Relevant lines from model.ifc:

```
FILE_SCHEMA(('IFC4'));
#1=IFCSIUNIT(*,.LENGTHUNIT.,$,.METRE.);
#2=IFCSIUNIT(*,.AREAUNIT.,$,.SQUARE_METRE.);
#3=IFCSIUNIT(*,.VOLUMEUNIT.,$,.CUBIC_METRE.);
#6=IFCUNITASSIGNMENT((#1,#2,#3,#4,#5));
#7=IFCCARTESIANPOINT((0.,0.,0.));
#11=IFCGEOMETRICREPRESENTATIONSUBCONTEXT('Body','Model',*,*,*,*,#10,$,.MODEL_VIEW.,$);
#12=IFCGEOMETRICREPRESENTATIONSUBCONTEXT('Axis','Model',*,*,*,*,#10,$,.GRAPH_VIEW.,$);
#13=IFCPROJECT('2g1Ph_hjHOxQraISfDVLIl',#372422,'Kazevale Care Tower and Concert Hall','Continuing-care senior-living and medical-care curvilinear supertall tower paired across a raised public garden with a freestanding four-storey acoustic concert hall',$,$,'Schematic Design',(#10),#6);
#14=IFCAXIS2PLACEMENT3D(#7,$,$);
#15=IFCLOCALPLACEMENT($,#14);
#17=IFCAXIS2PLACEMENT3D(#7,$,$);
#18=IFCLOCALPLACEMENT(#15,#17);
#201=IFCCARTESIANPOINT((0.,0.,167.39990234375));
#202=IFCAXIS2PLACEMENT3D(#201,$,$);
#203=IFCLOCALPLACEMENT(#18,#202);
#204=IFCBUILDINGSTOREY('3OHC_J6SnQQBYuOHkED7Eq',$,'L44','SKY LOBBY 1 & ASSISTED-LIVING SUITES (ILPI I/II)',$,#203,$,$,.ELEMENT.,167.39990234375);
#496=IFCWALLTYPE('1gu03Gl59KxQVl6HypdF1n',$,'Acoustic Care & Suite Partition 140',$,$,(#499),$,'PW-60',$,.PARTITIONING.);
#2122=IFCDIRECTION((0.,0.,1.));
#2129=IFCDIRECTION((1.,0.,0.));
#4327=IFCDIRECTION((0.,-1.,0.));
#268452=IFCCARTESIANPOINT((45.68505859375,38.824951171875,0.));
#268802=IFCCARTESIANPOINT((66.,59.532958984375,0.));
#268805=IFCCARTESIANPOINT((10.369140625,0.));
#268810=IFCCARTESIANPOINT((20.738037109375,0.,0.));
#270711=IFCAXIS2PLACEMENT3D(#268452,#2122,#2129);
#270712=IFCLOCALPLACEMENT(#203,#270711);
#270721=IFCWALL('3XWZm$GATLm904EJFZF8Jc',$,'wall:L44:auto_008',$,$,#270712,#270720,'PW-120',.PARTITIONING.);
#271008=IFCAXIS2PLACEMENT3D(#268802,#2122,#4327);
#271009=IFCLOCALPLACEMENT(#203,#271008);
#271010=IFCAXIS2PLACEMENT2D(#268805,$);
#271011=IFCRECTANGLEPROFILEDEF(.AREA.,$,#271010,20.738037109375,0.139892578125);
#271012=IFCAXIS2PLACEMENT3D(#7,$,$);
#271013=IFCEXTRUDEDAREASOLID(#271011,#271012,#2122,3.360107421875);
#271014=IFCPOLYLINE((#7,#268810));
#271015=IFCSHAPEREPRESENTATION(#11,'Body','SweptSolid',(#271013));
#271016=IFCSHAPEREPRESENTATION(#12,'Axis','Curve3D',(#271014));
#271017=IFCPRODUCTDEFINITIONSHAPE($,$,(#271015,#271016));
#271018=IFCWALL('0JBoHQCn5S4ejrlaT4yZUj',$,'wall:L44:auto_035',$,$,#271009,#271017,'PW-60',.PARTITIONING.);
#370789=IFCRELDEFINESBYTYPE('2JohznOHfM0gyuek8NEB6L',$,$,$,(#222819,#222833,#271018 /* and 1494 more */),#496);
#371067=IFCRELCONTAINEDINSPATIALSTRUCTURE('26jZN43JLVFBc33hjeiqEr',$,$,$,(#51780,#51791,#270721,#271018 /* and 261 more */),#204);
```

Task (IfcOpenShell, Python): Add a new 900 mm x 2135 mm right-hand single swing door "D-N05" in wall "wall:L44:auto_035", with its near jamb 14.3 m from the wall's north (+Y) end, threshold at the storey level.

```python
import numpy as np
import ifcopenshell
import ifcopenshell.api.feature
import ifcopenshell.api.geometry
import ifcopenshell.api.root
import ifcopenshell.api.spatial
import ifcopenshell.geom
import ifcopenshell.util.element
import ifcopenshell.util.placement
import ifcopenshell.util.representation
import ifcopenshell.util.shape
import ifcopenshell.util.unit

model = ifcopenshell.open("model.ifc")
unit_scale = ifcopenshell.util.unit.calculate_unit_scale(model)
settings = ifcopenshell.geom.settings()


def volume(element):
    """Net volume in cubic metres, openings subtracted."""
    shape = ifcopenshell.geom.create_shape(settings, element)
    return ifcopenshell.util.shape.get_volume(shape.geometry)


wall = model.by_id(271018)
storey = ifcopenshell.util.element.get_container(wall, ifc_class="IfcBuildingStorey")
context = ifcopenshell.util.representation.get_context(model, "Model", "Body", "MODEL_VIEW")
before = volume(wall)

width, height, from_end, sill = 0.9, 2.135, 14.3, 0.0  # metres

# The wall runs along its own X axis, and the end named is its -X end.
wall_shape = ifcopenshell.geom.create_shape(settings, wall)
x, y, z = ifcopenshell.util.shape.get_vertices(wall_shape.geometry).T
start = x.min() + from_end
face, thickness = float(y.min()), float(y.max() - y.min())
wall_matrix = ifcopenshell.util.placement.get_local_placement(wall.ObjectPlacement)
level = ifcopenshell.util.placement.get_local_placement(storey.ObjectPlacement)[2, 3]


def in_wall(x, y):
    """Placement at x, y metres in the wall's axes, at sill height."""
    matrix = wall_matrix.copy()
    matrix[:, 3] = wall_matrix @ np.array([x / unit_scale, y / unit_scale, 0.0, 1.0])
    matrix[2, 3] = level + sill / unit_scale
    return matrix


# Opening: a box that overshoots both wall faces by 50 mm.
opening = ifcopenshell.api.root.create_entity(model, ifc_class="IfcOpeningElement", predefined_type="OPENING")
box = ifcopenshell.api.geometry.add_wall_representation(
    model, context=context, length=width, height=height, thickness=thickness + 0.1
)
ifcopenshell.api.geometry.assign_representation(model, product=opening, representation=box)
ifcopenshell.api.geometry.edit_object_placement(model, product=opening, matrix=in_wall(start, face - 0.05), is_si=False)
ifcopenshell.api.feature.add_feature(model, feature=opening, element=wall)

door = ifcopenshell.api.root.create_entity(model, ifc_class="IfcDoor", name="D-N05", predefined_type="DOOR")
door.OverallWidth, door.OverallHeight = width / unit_scale, height / unit_scale
door.OperationType = "SINGLE_SWING_RIGHT"
body = ifcopenshell.api.geometry.add_door_representation(
    model,
    context=context,
    overall_width=door.OverallWidth,
    overall_height=door.OverallHeight,
    operation_type="SINGLE_SWING_RIGHT",
    lining_properties={"LiningDepth": thickness / unit_scale, "ThresholdDepth": thickness / unit_scale},
)
ifcopenshell.api.geometry.assign_representation(model, product=door, representation=body)
ifcopenshell.api.spatial.assign_container(model, products=[door], relating_structure=storey)
ifcopenshell.api.feature.add_filling(model, opening=opening, element=door)

# The lining spans the wall, so the door starts at the wall face.
ifcopenshell.api.geometry.edit_object_placement(model, product=door, matrix=in_wall(start, face), is_si=False)

after = volume(wall)

print(f"wall volume {before:.3f} -> {after:.3f} m3")

model.write("model_updated.ifc")
```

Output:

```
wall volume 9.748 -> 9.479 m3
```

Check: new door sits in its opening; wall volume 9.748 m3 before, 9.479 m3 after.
